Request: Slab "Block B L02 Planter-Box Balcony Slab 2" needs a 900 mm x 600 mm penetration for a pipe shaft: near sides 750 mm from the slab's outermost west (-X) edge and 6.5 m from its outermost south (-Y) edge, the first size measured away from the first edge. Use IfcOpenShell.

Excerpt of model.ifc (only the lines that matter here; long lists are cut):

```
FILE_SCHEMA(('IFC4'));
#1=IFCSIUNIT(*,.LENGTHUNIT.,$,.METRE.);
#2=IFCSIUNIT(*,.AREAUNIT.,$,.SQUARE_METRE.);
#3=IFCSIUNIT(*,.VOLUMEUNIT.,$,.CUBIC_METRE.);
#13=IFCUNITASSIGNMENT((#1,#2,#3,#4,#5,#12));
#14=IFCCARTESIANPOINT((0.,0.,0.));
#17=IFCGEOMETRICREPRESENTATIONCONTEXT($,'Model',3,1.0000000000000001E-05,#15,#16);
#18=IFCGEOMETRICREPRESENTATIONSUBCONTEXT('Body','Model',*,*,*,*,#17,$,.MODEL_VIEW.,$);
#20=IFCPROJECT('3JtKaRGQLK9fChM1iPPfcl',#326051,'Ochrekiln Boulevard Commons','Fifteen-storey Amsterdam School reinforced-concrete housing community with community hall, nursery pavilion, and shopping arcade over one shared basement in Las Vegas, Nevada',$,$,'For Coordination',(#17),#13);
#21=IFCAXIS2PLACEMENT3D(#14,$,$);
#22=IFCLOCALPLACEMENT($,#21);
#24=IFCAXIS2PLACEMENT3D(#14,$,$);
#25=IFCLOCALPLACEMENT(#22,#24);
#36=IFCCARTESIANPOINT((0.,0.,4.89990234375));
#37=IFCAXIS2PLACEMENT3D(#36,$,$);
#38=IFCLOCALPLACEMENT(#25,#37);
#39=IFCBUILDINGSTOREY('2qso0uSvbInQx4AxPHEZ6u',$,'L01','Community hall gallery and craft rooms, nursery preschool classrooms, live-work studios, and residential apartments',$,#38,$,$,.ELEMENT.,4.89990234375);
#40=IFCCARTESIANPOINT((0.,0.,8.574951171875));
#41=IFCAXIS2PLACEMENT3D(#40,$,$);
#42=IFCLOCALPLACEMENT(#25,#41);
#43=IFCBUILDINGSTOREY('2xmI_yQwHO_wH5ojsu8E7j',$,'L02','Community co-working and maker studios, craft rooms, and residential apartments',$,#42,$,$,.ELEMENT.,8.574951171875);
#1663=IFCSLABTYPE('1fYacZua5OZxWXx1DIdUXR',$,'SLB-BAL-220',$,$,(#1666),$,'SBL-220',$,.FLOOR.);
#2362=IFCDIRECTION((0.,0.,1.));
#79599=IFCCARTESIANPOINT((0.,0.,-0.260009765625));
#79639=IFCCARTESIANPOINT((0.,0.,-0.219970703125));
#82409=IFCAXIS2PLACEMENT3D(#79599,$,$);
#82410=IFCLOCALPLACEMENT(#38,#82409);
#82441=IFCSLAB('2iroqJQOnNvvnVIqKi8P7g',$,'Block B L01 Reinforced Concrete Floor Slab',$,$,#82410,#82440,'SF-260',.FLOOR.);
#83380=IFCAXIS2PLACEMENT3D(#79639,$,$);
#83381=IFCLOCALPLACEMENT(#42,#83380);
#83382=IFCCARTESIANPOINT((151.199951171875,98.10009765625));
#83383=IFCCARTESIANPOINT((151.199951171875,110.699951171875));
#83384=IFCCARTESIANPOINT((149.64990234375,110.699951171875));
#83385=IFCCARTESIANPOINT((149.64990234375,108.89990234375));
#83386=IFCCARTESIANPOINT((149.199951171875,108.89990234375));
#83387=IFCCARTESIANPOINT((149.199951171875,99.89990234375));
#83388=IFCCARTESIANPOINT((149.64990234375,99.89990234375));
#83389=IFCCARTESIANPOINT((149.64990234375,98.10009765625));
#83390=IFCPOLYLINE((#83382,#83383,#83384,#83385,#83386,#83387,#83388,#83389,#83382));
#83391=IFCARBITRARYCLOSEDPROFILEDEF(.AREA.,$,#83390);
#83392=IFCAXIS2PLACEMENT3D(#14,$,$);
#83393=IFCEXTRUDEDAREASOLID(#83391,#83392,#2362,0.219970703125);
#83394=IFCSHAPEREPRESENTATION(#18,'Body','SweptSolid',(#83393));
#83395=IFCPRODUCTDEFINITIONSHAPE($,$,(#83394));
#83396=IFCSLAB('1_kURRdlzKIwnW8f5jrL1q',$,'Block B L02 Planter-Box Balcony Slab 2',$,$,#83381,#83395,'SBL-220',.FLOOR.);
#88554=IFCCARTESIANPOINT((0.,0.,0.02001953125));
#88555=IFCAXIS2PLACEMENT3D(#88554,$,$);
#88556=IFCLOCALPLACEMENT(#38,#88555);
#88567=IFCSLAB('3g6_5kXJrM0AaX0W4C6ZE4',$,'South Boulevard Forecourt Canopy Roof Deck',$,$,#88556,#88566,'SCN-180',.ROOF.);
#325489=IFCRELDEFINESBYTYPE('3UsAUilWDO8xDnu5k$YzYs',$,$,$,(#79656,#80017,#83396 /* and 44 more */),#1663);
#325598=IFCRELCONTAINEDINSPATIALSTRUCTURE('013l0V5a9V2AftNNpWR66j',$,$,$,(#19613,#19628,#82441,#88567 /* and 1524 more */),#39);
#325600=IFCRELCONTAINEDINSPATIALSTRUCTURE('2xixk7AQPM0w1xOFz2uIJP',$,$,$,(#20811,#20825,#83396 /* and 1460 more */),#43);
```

```python
import numpy as np
import ifcopenshell
import ifcopenshell.api.feature
import ifcopenshell.api.geometry
import ifcopenshell.api.root
import ifcopenshell.geom
import ifcopenshell.util.placement
import ifcopenshell.util.representation
import ifcopenshell.util.shape
import ifcopenshell.util.unit

model = ifcopenshell.open("model.ifc")
unit_scale = ifcopenshell.util.unit.calculate_unit_scale(model)
settings = ifcopenshell.geom.settings()


def volume(element):
    """Net volume in cubic metres, openings subtracted."""
    shape = ifcopenshell.geom.create_shape(settings, element)
    return ifcopenshell.util.shape.get_volume(shape.geometry)


slab = model.by_guid("1_kURRdlzKIwnW8f5jrL1q")
before = volume(slab)

# Extent in the slab's own axes, in metres. The edges named are its -X and -Y sides.
slab_shape = ifcopenshell.geom.create_shape(settings, slab)
vertices = ifcopenshell.util.shape.get_vertices(slab_shape.geometry)
x_min, y_min, bottom = vertices.min(axis=0)
top = vertices[:, 2].max()

opening = ifcopenshell.api.root.create_entity(model, ifc_class="IfcOpeningElement", name="Pipe shaft opening", predefined_type="OPENING")
context = ifcopenshell.util.representation.get_context(model, "Model", "Body", "MODEL_VIEW")
width, depth = 0.9, 0.6
outline = [(0.0, 0.0), (width, 0.0), (width, depth), (0.0, depth), (0.0, 0.0)]
# Overshoot both faces by 50 mm so the cut is clean.
shape = ifcopenshell.api.geometry.add_slab_representation(
    model, context=context, depth=top - bottom + 0.1, polyline=outline
)
ifcopenshell.api.geometry.assign_representation(model, product=opening, representation=shape)

matrix = ifcopenshell.util.placement.get_local_placement(slab.ObjectPlacement)
matrix[:, 3] = matrix @ np.append(np.array([x_min + 0.75, y_min + 6.5, bottom - 0.05]) / unit_scale, 1.0)
ifcopenshell.api.geometry.edit_object_placement(model, product=opening, matrix=matrix, is_si=False)
ifcopenshell.api.feature.add_feature(model, feature=opening, element=slab)

after = volume(slab)

print(f"slab volume {before:.3f} -> {after:.3f} m3")

model.write("model-out.ifc")
```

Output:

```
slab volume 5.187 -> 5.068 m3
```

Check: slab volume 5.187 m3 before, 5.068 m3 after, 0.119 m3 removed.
